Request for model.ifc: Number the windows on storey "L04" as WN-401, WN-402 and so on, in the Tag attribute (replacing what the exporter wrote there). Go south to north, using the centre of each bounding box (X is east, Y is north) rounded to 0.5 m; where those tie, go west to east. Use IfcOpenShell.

First a look at what the model holds.

```python
import ifcopenshell
import ifcopenshell.util.element
import ifcopenshell.util.placement

model = ifcopenshell.open("model.ifc")
print(model.schema)
storey = next(s for s in model.by_type("IfcBuildingStorey") if s.Name == "L04")
windows = [e for e in ifcopenshell.util.element.get_decomposition(storey) if e.is_a("IfcWindow")]
for e in sorted(windows, key=lambda e: e.id()):
    origin = ifcopenshell.util.placement.get_local_placement(e.ObjectPlacement)[:3, 3]
    print(e.id(), e.Tag, e.Name, origin.round(2) + 0.0, sep=" | ")
```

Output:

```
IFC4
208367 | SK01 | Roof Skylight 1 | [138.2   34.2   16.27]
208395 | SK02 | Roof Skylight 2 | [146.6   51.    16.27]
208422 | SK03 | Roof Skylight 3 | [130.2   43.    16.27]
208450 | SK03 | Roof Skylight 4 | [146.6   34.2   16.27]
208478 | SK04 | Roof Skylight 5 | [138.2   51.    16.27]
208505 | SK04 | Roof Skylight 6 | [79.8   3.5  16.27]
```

```python
import ifcopenshell
import ifcopenshell.geom
import ifcopenshell.util.element
import ifcopenshell.util.shape

model = ifcopenshell.open("model.ifc")
settings = ifcopenshell.geom.settings()
settings.set("use-world-coords", True)


def centre(element):
    shape = ifcopenshell.geom.create_shape(settings, element)
    return ifcopenshell.util.shape.get_bbox_centroid(shape.geometry)


storey = next(s for s in model.by_type("IfcBuildingStorey") if s.Name == "L04")
windows = [e for e in ifcopenshell.util.element.get_decomposition(storey) if e.is_a("IfcWindow")]

# Insertion points can sit at a corner or the storey origin, so sort by the geometry (in metres).
centres = {e: centre(e) for e in windows}
windows.sort(key=lambda e: (round(centres[e][1] / 0.5), centres[e][0]))

for i, e in enumerate(windows, start=1):
    number = f"WN-4{i:02d}"
    e.Tag = number
    print(e.id(), number)

model.write("model_v2.ifc")
```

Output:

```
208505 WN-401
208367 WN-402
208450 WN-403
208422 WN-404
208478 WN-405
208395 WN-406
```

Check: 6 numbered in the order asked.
